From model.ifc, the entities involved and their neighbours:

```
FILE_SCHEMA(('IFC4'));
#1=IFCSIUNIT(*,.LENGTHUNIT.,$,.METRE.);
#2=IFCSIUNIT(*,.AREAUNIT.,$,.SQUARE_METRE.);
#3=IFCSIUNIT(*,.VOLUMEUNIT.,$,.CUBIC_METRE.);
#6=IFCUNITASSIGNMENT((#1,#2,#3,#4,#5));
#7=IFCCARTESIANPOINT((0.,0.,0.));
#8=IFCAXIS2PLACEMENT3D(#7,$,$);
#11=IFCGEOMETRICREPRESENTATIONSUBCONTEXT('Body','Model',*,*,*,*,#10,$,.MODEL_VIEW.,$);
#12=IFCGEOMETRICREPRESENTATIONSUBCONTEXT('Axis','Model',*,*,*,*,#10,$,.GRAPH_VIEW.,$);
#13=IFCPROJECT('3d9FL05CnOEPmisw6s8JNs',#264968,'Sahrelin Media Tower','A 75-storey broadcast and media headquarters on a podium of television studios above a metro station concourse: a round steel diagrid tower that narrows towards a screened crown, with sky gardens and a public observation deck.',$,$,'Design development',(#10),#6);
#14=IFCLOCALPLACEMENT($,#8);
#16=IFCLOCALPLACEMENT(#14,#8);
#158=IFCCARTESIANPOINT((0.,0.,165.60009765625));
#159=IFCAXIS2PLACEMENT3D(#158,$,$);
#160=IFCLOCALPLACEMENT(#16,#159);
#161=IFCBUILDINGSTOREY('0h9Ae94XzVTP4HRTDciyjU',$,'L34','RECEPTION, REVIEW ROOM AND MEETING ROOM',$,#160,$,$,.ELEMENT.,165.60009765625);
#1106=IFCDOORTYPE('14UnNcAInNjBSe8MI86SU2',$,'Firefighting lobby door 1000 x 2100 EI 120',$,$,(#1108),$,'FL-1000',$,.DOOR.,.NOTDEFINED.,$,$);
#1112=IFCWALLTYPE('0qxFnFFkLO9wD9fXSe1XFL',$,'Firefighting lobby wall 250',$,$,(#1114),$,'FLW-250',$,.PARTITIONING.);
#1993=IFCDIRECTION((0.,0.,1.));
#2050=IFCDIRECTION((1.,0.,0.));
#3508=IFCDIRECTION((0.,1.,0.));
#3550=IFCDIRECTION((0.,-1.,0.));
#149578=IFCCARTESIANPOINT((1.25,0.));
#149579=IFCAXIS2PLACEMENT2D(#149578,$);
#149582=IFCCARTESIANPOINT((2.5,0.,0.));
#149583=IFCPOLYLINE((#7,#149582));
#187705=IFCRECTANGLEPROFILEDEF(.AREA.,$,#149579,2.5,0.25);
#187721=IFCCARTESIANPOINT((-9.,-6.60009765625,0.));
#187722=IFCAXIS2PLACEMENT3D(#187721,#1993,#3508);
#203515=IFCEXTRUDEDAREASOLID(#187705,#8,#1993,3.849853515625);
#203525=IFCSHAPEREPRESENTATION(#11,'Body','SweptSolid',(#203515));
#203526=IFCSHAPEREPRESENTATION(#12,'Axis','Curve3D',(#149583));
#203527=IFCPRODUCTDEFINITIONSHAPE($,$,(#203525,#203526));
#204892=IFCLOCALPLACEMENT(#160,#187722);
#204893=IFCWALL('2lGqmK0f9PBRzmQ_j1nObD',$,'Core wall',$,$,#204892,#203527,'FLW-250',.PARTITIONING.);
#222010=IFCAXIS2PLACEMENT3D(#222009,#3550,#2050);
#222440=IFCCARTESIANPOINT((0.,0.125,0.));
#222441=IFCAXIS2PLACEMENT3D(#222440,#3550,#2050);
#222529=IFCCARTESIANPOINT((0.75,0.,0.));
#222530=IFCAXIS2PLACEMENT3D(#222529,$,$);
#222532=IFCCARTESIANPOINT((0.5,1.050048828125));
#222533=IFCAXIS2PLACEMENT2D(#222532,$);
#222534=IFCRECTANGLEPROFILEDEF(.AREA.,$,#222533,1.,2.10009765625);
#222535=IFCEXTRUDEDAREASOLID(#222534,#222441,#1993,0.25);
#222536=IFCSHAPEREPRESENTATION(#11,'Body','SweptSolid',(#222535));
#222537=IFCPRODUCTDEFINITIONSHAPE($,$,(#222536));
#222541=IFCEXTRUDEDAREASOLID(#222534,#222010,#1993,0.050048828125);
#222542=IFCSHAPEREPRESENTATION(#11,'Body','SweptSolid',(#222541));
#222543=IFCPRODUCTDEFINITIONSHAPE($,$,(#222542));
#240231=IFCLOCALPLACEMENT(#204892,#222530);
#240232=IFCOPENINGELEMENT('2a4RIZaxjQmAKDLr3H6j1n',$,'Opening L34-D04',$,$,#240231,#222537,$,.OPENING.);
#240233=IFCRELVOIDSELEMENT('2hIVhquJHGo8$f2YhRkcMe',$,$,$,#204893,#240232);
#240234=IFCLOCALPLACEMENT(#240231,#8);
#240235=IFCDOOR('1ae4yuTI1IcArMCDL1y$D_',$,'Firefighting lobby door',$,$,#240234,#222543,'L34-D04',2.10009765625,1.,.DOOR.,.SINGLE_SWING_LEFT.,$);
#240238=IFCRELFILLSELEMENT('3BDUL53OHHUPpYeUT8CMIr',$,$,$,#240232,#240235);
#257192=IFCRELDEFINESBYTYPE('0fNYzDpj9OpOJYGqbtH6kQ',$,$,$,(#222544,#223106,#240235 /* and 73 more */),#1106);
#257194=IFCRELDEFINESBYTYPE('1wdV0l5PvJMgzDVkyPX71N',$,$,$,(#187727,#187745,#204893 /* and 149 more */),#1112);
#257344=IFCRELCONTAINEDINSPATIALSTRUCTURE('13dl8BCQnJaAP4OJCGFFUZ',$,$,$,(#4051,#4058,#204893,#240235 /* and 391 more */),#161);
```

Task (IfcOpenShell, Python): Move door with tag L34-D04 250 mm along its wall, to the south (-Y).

```python
import ifcopenshell
import ifcopenshell.api.geometry
import ifcopenshell.util.placement

model = ifcopenshell.open("model.ifc")

door = model.by_id(240235)
opening = door.FillsVoids[0].RelatingOpeningElement
wall = opening.VoidsElements[0].RelatingBuildingElement

wall_matrix = ifcopenshell.util.placement.get_local_placement(wall.ObjectPlacement)
shift = wall_matrix[:3, 0] * -0.25
before = ifcopenshell.util.placement.get_local_placement(door.ObjectPlacement)[:3, 3].copy()

# The door is placed relative to its opening, so it follows when the opening moves.
matrix = ifcopenshell.util.placement.get_local_placement(opening.ObjectPlacement)
matrix[:3, 3] += shift
ifcopenshell.api.geometry.edit_object_placement(
    model, product=opening, matrix=matrix, is_si=False, should_transform_children=True
)

after = ifcopenshell.util.placement.get_local_placement(door.ObjectPlacement)[:3, 3]
print("door moved by", (after - before).round(3) + 0.0)

model.write("model_edited.ifc")
```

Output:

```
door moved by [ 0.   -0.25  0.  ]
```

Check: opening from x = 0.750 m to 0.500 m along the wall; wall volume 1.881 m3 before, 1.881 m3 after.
